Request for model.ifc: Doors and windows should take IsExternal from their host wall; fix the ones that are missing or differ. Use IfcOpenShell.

First a look at what the model holds.

```python
import ifcopenshell
import ifcopenshell.util.element

model = ifcopenshell.open("model.ifc")
print(model.schema)
seen = {}
for e in model.by_type("IfcDoor") + model.by_type("IfcWindow"):
    if not e.FillsVoids:
        continue
    host = e.FillsVoids[0].RelatingOpeningElement.VoidsElements[0].RelatingBuildingElement
    own = ifcopenshell.util.element.get_pset(e, f"Pset_{e.is_a()[3:].removesuffix('StandardCase')}Common", "IsExternal")
    wall = ifcopenshell.util.element.get_pset(host, "Pset_WallCommon", "IsExternal")
    seen[e.is_a(), own, wall] = seen.get((e.is_a(), own, wall), 0) + 1
for (cls, own, wall), count in sorted(seen.items(), key=str):
    print(count, cls, "IsExternal:", own, "| host wall:", wall)
```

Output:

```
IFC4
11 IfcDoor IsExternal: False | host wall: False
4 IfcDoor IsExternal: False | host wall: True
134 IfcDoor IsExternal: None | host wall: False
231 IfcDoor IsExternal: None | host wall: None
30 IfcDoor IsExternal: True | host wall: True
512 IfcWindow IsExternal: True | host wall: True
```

```python
import ifcopenshell
import ifcopenshell.api.pset
import ifcopenshell.util.element

model = ifcopenshell.open("model.ifc")

count = 0
for ifc_class, pset_name in (("IfcDoor", "Pset_DoorCommon"), ("IfcWindow", "Pset_WindowCommon")):
    for e in model.by_type(ifc_class):
        if not e.FillsVoids:
            continue
        host = e.FillsVoids[0].RelatingOpeningElement.VoidsElements[0].RelatingBuildingElement
        external = ifcopenshell.util.element.get_pset(host, "Pset_WallCommon", "IsExternal")
        if external is None or ifcopenshell.util.element.get_pset(e, pset_name, "IsExternal") == external:
            continue
        pset = ifcopenshell.api.pset.add_pset(model, product=e, name=pset_name)
        ifcopenshell.api.pset.edit_pset(model, pset=pset, properties={"IsExternal": external})
        count += 1

print(count, "updated")

model.write("model_edited.ifc")
```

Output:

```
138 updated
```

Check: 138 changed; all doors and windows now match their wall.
